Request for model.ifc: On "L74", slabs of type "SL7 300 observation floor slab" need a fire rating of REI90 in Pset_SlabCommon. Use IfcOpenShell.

First a look at what the model holds.

```python
import ifcopenshell
import ifcopenshell.util.element

model = ifcopenshell.open("model.ifc")
print(model.schema)
storey = next(s for s in model.by_type("IfcBuildingStorey") if s.Name == "L74")
slabs = [e for e in ifcopenshell.util.element.get_decomposition(storey) if e.is_a("IfcSlab")]
seen = {}
for e in slabs:
    element_type = ifcopenshell.util.element.get_type(e)
    key = (element_type.Name if element_type != e and element_type else None, ifcopenshell.util.element.get_pset(e, "Pset_SlabCommon", "FireRating"))
    seen[key] = seen.get(key, 0) + 1
for (name, value), count in sorted(seen.items(), key=str):
    print(count, "x", name, "|", value)
```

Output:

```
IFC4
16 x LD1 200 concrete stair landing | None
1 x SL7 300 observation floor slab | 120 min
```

```python
import ifcopenshell
import ifcopenshell.api.pset
import ifcopenshell.util.element

model = ifcopenshell.open("model.ifc")

storey = next(s for s in model.by_type("IfcBuildingStorey") if s.Name == "L74")
slabs = [e for e in ifcopenshell.util.element.get_decomposition(storey) if e.is_a("IfcSlab")]

count = 0
for e in slabs:
    element_type = ifcopenshell.util.element.get_type(e)
    if element_type in (None, e) or element_type.Name != "SL7 300 observation floor slab":
        continue
    # add_pset returns the element's existing set when there is one.
    pset = ifcopenshell.api.pset.add_pset(model, product=e, name="Pset_SlabCommon")
    ifcopenshell.api.pset.edit_pset(model, pset=pset, properties={"FireRating": "REI90"})
    count += 1

print(count, "slabs updated")

model.write("model_v2.ifc")
```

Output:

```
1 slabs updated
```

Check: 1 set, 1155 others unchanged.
